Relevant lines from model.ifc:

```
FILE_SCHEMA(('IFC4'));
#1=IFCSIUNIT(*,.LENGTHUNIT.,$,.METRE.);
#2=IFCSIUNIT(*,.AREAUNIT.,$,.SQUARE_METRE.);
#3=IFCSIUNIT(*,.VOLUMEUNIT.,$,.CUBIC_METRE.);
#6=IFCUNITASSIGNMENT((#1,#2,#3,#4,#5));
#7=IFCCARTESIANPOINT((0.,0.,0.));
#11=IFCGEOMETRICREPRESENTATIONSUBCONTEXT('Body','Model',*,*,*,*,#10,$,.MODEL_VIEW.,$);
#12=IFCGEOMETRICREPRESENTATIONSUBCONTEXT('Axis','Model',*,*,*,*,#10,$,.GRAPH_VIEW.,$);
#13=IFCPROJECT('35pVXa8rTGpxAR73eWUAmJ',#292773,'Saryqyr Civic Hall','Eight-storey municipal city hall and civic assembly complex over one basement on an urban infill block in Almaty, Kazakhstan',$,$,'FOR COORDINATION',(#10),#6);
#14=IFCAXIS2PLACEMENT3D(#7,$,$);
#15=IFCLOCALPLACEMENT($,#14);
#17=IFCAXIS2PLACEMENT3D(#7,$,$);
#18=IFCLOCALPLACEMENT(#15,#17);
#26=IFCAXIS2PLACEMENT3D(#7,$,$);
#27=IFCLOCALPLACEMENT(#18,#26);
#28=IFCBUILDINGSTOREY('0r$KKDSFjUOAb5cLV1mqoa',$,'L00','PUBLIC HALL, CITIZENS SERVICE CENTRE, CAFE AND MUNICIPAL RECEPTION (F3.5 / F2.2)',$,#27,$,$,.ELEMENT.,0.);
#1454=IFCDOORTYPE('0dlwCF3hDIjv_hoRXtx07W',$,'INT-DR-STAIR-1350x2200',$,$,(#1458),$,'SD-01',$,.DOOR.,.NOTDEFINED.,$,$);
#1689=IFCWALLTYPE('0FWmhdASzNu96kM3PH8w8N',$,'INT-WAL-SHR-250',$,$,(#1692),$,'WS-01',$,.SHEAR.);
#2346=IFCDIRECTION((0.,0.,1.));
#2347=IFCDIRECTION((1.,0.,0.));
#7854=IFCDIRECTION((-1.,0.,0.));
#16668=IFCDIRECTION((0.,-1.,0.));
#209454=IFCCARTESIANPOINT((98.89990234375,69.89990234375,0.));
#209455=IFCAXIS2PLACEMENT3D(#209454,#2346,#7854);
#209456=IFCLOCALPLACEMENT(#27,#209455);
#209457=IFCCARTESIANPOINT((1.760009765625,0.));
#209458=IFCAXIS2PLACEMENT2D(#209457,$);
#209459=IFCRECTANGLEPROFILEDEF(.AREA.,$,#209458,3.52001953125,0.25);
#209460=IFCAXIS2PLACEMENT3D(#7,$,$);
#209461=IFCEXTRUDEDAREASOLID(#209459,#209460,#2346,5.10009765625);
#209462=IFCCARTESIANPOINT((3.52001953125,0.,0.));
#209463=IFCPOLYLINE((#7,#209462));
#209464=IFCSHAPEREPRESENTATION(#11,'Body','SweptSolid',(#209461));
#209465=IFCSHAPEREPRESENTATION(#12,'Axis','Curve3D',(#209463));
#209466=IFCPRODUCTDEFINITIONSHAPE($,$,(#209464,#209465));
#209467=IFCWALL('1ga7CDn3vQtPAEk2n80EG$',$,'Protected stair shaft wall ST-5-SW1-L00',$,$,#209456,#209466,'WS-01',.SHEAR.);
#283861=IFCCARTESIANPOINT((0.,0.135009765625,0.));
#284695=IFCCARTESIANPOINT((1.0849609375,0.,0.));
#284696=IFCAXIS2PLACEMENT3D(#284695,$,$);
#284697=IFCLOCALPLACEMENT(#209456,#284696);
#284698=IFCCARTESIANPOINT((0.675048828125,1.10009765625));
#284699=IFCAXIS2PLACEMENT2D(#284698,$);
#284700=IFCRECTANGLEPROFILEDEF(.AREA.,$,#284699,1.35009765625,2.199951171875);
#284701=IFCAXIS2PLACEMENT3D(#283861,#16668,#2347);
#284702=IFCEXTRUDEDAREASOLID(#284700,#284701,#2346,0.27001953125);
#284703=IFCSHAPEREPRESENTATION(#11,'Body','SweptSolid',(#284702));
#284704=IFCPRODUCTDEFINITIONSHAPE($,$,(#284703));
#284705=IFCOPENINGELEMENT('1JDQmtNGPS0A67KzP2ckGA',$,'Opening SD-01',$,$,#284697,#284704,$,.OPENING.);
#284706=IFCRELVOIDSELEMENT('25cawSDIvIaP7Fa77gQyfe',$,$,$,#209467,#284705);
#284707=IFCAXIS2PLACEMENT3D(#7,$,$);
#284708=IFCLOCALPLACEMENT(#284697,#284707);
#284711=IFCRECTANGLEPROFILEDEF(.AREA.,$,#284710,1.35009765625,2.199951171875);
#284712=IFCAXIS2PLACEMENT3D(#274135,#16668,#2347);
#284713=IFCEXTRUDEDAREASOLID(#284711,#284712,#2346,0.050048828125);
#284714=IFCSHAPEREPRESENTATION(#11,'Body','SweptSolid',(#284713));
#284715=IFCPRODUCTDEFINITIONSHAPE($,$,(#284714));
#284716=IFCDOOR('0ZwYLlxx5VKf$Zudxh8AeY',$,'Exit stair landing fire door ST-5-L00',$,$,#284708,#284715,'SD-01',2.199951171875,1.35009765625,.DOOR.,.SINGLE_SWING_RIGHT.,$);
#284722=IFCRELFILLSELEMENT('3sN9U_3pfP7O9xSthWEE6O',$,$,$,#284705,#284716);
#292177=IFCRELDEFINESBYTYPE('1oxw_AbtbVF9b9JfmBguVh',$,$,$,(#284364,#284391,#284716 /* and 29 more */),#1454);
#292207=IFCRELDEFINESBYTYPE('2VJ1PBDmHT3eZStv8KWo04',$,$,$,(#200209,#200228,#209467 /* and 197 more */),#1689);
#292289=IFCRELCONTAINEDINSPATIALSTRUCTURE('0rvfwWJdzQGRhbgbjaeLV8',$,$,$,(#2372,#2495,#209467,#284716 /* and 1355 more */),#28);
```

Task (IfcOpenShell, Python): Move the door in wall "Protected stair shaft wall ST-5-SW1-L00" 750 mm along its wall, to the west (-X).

```python
import ifcopenshell
import ifcopenshell.api.geometry
import ifcopenshell.util.placement

model = ifcopenshell.open("model.ifc")

door = model.by_id(284716)
opening = door.FillsVoids[0].RelatingOpeningElement
wall = opening.VoidsElements[0].RelatingBuildingElement

wall_matrix = ifcopenshell.util.placement.get_local_placement(wall.ObjectPlacement)
shift = wall_matrix[:3, 0] * 0.75
before = ifcopenshell.util.placement.get_local_placement(door.ObjectPlacement)[:3, 3].copy()

# The door is placed relative to its opening, so it follows when the opening moves.
matrix = ifcopenshell.util.placement.get_local_placement(opening.ObjectPlacement)
matrix[:3, 3] += shift
ifcopenshell.api.geometry.edit_object_placement(
    model, product=opening, matrix=matrix, is_si=False, should_transform_children=True
)

after = ifcopenshell.util.placement.get_local_placement(door.ObjectPlacement)[:3, 3]
print("door moved by", (after - before).round(3) + 0.0)

model.write("model_updated.ifc")
```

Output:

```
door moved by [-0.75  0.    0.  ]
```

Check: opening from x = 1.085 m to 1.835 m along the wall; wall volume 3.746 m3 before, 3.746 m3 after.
